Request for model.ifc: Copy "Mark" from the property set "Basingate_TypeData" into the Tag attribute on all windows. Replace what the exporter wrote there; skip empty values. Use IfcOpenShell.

First a look at what the model holds.

```python
import ifcopenshell
import ifcopenshell.util.element

model = ifcopenshell.open("model.ifc")
print(model.schema)
windows = model.by_type("IfcWindow")
print(len(windows), "windows")
for e in windows[:8]:
    source = ifcopenshell.util.element.get_pset(e, "Basingate_TypeData", "Mark")
    target = e.Tag
    print(e.id(), repr(source), repr(target), sep=" | ")
```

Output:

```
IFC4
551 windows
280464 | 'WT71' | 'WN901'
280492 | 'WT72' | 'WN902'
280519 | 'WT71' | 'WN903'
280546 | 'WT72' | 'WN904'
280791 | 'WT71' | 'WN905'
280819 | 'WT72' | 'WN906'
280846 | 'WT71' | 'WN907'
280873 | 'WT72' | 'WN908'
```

```python
import ifcopenshell
import ifcopenshell.util.element

model = ifcopenshell.open("model.ifc")

count = 0
for e in model.by_type("IfcWindow"):
    value = ifcopenshell.util.element.get_pset(e, "Basingate_TypeData", "Mark")
    current = e.Tag
    if not value or not value.strip() or current == value:
        continue
    e.Tag = value
    count += 1

print(count, "windows updated")

model.write("model_updated.ifc")
```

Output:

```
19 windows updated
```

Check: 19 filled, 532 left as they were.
